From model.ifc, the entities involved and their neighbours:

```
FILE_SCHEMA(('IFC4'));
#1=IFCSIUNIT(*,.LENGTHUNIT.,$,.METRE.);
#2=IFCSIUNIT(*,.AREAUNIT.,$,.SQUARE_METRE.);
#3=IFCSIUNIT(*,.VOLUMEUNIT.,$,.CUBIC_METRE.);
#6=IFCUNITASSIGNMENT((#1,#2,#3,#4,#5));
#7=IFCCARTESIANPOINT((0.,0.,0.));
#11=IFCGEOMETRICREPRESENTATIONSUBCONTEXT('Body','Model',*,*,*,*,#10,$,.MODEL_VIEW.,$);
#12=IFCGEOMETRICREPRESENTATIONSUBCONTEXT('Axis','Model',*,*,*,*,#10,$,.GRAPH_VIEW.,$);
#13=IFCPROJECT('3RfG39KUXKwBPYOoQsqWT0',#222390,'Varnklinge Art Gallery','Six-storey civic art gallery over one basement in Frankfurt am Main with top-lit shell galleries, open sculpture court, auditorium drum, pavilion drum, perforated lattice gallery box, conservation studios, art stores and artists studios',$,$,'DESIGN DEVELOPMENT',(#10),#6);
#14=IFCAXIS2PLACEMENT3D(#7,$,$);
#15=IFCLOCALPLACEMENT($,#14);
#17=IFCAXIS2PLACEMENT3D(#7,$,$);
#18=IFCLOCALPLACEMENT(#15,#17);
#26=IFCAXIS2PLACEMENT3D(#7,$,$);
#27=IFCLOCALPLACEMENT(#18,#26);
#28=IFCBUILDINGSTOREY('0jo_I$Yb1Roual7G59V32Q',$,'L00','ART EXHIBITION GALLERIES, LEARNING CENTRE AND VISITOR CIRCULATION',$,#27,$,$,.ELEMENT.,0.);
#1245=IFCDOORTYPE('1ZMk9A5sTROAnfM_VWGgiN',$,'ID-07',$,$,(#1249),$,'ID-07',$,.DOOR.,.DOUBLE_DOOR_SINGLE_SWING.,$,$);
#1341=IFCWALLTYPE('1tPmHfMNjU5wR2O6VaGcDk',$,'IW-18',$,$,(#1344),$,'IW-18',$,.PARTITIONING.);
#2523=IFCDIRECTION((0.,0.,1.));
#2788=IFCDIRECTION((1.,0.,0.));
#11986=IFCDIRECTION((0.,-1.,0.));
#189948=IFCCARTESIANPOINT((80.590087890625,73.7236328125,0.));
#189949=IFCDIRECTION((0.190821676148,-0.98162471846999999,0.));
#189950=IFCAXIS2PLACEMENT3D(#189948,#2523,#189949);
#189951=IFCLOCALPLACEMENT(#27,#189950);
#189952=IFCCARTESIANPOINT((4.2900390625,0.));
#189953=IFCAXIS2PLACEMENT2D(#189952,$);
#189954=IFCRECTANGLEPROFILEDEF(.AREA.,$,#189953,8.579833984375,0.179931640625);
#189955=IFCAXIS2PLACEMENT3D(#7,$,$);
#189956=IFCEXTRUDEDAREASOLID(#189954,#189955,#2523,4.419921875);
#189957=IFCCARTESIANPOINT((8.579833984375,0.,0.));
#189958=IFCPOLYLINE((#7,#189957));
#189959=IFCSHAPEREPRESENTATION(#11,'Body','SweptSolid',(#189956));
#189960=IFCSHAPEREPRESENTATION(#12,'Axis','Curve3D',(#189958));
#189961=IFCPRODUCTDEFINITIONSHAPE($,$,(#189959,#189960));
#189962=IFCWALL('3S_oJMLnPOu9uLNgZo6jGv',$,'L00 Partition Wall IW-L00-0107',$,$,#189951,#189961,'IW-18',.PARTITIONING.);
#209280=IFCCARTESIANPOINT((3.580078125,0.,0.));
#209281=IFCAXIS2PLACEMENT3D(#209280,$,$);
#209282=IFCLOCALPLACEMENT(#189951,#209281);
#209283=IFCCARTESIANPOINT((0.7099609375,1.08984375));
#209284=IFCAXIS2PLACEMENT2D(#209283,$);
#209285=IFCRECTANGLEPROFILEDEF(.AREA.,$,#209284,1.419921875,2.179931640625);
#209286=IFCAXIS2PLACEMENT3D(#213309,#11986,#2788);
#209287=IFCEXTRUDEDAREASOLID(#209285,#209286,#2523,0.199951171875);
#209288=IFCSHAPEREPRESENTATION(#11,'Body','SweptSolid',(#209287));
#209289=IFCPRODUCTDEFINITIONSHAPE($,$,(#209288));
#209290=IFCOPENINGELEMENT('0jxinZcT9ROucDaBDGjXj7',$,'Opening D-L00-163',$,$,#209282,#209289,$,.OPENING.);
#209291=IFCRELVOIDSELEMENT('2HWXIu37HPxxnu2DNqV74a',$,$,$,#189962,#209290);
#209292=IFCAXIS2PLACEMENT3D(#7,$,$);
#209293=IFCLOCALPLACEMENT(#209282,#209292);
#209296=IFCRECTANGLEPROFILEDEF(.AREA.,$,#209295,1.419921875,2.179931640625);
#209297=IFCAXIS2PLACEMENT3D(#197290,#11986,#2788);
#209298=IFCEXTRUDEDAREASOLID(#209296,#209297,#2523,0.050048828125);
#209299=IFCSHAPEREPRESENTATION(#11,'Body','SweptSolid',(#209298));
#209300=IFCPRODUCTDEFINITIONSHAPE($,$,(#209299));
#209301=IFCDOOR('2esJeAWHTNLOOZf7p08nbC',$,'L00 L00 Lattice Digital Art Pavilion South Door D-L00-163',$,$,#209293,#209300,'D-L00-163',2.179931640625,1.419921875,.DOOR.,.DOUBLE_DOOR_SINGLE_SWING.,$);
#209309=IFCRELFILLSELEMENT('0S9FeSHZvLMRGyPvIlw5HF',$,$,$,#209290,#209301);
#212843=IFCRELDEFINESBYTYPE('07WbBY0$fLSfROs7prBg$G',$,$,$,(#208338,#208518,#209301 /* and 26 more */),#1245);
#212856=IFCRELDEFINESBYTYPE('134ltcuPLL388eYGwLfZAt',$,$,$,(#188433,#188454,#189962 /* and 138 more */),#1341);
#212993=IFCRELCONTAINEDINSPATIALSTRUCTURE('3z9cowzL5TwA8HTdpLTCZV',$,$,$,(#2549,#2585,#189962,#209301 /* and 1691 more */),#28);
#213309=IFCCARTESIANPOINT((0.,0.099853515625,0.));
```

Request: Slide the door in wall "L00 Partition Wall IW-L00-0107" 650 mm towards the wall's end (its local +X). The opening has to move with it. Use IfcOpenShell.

```python
import ifcopenshell
import ifcopenshell.api.geometry
import ifcopenshell.util.placement
import ifcopenshell.util.unit

model = ifcopenshell.open("model.ifc")
unit_scale = ifcopenshell.util.unit.calculate_unit_scale(model)

door = model.by_guid("2esJeAWHTNLOOZf7p08nbC")
opening = door.FillsVoids[0].RelatingOpeningElement
wall = opening.VoidsElements[0].RelatingBuildingElement

wall_matrix = ifcopenshell.util.placement.get_local_placement(wall.ObjectPlacement)
shift = wall_matrix[:3, 0] * 0.65 / unit_scale
before = ifcopenshell.util.placement.get_local_placement(door.ObjectPlacement)[:3, 3].copy()

# The door is placed relative to its opening, so it follows when the opening moves.
matrix = ifcopenshell.util.placement.get_local_placement(opening.ObjectPlacement)
matrix[:3, 3] += shift
ifcopenshell.api.geometry.edit_object_placement(
    model, product=opening, matrix=matrix, is_si=False, should_transform_children=True
)

after = ifcopenshell.util.placement.get_local_placement(door.ObjectPlacement)[:3, 3]
print("door moved by", (after - before).round(3) + 0.0)

model.write("model_edited.ifc")
```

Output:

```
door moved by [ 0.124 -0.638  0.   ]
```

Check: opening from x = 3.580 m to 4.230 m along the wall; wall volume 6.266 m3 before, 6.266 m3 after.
